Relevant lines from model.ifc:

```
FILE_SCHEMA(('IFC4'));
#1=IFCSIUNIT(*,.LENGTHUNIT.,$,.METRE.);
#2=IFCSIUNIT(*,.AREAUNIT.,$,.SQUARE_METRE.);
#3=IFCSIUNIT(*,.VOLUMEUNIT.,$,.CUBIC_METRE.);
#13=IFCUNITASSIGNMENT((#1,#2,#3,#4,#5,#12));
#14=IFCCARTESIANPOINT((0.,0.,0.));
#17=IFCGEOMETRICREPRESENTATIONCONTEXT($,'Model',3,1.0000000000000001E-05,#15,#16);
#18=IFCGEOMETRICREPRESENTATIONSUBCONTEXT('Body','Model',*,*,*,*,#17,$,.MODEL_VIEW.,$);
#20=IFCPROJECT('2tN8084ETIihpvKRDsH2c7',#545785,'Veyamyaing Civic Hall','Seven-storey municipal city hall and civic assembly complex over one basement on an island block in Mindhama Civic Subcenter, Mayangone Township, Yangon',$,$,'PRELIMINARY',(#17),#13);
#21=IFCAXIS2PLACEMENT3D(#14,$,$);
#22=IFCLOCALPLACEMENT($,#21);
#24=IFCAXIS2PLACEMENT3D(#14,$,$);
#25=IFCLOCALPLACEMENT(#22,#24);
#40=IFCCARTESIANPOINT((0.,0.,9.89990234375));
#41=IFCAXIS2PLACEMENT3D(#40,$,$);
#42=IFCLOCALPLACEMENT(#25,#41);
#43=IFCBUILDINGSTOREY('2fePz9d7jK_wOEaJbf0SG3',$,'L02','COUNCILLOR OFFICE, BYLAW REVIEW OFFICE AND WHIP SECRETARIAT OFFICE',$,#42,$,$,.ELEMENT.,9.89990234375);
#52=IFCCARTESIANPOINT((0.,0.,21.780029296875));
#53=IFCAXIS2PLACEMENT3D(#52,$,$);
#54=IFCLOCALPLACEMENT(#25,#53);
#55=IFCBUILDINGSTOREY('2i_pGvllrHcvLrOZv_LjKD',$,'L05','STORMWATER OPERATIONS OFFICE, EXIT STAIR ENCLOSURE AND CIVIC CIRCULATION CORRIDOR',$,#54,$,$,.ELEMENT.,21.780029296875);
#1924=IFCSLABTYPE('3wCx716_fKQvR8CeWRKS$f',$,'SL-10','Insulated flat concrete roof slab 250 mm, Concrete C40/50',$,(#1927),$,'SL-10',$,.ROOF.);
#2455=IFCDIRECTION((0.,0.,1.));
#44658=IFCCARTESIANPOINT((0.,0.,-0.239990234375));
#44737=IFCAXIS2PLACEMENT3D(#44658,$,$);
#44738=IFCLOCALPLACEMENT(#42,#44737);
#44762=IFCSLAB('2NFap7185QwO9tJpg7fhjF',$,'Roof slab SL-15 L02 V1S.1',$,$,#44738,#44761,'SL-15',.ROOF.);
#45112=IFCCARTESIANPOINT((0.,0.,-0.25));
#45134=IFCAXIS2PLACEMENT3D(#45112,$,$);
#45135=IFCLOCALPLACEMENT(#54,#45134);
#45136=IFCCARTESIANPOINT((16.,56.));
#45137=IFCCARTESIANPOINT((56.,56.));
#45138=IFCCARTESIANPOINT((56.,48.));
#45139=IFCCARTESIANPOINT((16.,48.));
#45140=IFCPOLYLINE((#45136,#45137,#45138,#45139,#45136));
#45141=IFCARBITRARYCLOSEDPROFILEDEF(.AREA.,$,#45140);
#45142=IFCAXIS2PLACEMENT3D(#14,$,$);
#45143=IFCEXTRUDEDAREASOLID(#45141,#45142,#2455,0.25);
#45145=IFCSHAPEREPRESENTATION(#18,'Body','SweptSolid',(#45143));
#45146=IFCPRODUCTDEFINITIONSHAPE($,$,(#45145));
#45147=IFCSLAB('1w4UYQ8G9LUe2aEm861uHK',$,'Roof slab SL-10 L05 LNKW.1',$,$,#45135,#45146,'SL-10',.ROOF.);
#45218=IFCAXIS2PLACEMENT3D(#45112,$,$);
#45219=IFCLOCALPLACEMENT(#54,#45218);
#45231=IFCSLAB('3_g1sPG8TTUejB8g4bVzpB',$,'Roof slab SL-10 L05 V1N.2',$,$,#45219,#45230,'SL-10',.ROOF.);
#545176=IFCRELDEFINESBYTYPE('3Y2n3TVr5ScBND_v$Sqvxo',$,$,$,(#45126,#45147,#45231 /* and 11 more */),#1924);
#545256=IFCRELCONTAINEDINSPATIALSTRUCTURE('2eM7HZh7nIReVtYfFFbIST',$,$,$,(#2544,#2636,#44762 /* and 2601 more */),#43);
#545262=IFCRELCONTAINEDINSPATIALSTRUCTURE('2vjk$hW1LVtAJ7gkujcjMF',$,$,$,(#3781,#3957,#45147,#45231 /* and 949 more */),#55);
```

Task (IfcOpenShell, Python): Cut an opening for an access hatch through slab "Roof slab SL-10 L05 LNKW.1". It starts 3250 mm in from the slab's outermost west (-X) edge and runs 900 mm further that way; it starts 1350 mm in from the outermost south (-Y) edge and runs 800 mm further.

```python
import numpy as np
import ifcopenshell
import ifcopenshell.api.feature
import ifcopenshell.api.geometry
import ifcopenshell.api.root
import ifcopenshell.geom
import ifcopenshell.util.placement
import ifcopenshell.util.representation
import ifcopenshell.util.shape
import ifcopenshell.util.unit

model = ifcopenshell.open("model.ifc")
unit_scale = ifcopenshell.util.unit.calculate_unit_scale(model)
settings = ifcopenshell.geom.settings()


def volume(element):
    """Net volume in cubic metres, openings subtracted."""
    shape = ifcopenshell.geom.create_shape(settings, element)
    return ifcopenshell.util.shape.get_volume(shape.geometry)


slab = model.by_guid("1w4UYQ8G9LUe2aEm861uHK")
before = volume(slab)

# Extent in the slab's own axes, in metres. The edges named are its -X and -Y sides.
slab_shape = ifcopenshell.geom.create_shape(settings, slab)
vertices = ifcopenshell.util.shape.get_vertices(slab_shape.geometry)
x_min, y_min, bottom = vertices.min(axis=0)
top = vertices[:, 2].max()

opening = ifcopenshell.api.root.create_entity(model, ifc_class="IfcOpeningElement", name="Access hatch opening", predefined_type="OPENING")
context = ifcopenshell.util.representation.get_context(model, "Model", "Body", "MODEL_VIEW")
width, depth = 0.9, 0.8
outline = [(0.0, 0.0), (width, 0.0), (width, depth), (0.0, depth), (0.0, 0.0)]
# Overshoot both faces by 50 mm so the cut is clean.
shape = ifcopenshell.api.geometry.add_slab_representation(
    model, context=context, depth=top - bottom + 0.1, polyline=outline
)
ifcopenshell.api.geometry.assign_representation(model, product=opening, representation=shape)

matrix = ifcopenshell.util.placement.get_local_placement(slab.ObjectPlacement)
matrix[:, 3] = matrix @ np.append(np.array([x_min + 3.25, y_min + 1.35, bottom - 0.05]) / unit_scale, 1.0)
ifcopenshell.api.geometry.edit_object_placement(model, product=opening, matrix=matrix, is_si=False)
ifcopenshell.api.feature.add_feature(model, feature=opening, element=slab)

after = volume(slab)

print(f"slab volume {before:.3f} -> {after:.3f} m3")

model.write("model_rev.ifc")
```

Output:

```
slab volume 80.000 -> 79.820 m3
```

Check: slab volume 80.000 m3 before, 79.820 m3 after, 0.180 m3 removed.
